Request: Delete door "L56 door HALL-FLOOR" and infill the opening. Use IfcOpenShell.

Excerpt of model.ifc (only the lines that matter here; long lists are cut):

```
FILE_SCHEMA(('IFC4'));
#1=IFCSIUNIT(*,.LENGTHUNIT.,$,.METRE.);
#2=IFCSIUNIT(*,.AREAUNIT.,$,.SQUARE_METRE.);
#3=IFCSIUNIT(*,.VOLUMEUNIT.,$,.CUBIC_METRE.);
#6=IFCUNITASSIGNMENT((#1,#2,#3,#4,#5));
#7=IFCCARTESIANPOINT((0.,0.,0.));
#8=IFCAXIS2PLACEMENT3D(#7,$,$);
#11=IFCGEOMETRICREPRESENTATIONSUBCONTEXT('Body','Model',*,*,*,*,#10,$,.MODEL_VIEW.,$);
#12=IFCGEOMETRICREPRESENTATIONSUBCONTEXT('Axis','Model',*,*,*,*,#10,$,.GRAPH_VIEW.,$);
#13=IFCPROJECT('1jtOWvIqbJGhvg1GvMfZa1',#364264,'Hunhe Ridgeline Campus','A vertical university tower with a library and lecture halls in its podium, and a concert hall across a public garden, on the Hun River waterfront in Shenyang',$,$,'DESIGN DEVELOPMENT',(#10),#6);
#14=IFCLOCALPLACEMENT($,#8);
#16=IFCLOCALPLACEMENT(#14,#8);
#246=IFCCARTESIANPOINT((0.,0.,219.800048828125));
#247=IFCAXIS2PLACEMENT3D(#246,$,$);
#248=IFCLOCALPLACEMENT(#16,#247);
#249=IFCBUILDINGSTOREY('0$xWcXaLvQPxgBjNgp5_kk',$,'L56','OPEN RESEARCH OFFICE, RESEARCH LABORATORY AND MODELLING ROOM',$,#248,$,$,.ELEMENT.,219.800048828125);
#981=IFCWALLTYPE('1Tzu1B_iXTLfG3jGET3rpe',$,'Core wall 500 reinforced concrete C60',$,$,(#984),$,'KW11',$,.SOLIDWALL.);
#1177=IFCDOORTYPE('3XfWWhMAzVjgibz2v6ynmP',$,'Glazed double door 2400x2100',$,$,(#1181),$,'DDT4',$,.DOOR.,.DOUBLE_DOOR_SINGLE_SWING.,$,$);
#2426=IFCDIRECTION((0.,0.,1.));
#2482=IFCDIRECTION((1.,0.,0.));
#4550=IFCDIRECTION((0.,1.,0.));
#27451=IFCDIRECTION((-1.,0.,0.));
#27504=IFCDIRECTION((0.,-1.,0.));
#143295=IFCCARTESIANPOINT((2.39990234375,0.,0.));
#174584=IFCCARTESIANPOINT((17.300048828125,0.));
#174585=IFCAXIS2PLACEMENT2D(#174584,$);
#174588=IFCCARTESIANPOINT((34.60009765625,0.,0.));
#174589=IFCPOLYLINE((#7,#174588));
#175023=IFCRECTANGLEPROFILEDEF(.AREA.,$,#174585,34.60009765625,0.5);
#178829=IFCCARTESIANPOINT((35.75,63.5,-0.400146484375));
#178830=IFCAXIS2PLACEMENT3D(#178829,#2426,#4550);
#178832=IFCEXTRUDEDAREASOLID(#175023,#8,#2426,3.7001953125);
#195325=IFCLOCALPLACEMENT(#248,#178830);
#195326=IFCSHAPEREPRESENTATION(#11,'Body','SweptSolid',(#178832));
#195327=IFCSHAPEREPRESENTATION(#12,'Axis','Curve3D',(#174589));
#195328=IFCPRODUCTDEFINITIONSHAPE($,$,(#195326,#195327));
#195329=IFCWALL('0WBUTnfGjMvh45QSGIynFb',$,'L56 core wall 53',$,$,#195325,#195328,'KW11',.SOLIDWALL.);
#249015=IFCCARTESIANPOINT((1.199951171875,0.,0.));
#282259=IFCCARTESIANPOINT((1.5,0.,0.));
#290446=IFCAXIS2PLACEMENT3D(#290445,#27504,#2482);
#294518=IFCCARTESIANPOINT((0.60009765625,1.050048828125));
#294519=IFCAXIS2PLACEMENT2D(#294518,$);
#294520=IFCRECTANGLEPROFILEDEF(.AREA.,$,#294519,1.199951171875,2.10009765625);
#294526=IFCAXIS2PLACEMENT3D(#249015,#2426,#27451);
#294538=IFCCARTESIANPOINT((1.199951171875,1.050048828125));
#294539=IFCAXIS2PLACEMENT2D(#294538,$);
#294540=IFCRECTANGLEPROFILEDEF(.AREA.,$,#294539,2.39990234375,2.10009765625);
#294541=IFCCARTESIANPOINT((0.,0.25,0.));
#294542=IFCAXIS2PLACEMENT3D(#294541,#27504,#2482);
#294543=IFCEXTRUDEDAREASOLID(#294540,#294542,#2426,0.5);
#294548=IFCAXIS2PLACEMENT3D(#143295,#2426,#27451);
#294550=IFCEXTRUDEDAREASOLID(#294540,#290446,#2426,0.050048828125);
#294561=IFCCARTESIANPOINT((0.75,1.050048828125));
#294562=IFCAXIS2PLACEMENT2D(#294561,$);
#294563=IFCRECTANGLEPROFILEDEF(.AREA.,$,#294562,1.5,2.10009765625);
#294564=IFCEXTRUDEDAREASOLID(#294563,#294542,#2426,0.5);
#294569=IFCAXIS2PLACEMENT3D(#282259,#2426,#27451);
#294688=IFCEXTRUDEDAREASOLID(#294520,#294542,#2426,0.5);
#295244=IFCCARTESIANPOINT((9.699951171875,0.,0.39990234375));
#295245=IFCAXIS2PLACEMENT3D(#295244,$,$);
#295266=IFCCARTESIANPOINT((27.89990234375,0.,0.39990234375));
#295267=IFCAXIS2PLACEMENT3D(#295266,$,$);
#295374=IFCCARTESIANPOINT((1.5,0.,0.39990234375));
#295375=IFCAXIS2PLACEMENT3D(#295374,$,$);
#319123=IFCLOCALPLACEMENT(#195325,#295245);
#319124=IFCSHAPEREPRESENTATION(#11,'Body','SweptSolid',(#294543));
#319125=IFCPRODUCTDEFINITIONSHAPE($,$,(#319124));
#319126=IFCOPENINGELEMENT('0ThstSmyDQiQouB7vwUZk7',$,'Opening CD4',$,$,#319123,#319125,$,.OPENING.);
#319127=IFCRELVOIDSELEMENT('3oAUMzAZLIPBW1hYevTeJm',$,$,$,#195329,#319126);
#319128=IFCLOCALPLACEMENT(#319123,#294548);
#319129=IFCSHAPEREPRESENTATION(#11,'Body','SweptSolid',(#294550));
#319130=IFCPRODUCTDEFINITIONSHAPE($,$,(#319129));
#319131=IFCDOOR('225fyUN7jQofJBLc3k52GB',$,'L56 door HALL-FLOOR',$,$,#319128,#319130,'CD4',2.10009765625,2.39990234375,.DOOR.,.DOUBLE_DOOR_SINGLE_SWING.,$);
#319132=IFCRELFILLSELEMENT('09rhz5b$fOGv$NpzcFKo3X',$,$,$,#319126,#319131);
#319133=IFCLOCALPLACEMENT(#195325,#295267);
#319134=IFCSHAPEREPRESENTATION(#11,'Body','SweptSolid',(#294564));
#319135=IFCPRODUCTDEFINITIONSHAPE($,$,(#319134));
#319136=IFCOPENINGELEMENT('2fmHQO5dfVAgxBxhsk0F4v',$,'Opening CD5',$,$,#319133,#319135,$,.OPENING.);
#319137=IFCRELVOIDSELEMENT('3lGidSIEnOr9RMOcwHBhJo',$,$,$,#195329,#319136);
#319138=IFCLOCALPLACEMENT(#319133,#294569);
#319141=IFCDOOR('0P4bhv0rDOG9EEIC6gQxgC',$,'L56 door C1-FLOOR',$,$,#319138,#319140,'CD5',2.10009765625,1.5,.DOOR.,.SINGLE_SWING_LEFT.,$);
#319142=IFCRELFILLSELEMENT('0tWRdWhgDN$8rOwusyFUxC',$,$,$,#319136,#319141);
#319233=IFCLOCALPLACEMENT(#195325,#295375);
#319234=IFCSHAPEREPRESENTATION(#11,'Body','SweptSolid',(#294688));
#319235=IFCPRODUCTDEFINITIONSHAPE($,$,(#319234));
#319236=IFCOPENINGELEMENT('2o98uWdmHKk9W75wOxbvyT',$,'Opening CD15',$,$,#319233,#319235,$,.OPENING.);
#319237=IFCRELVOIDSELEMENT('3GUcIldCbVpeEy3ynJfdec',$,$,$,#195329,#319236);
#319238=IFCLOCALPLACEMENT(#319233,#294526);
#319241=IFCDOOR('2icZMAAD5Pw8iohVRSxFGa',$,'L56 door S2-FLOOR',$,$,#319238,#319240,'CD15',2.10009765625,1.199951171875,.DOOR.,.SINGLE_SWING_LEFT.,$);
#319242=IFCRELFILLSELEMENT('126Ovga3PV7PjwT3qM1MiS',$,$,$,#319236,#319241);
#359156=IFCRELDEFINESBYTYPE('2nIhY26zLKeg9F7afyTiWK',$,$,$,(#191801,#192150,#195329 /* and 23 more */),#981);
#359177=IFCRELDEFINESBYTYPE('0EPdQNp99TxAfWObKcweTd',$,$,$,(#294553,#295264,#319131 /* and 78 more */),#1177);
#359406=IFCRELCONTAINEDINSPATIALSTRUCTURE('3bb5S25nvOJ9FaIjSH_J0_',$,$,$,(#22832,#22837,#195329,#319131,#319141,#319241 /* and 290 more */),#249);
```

```python
import ifcopenshell
import ifcopenshell.api.feature
import ifcopenshell.api.root
import ifcopenshell.geom
import ifcopenshell.util.shape

model = ifcopenshell.open("model.ifc")
settings = ifcopenshell.geom.settings()


def volume(element):
    """Net volume in cubic metres, openings subtracted."""
    shape = ifcopenshell.geom.create_shape(settings, element)
    return ifcopenshell.util.shape.get_volume(shape.geometry)


door = model.by_guid("225fyUN7jQofJBLc3k52GB")
opening = door.FillsVoids[0].RelatingOpeningElement
wall = opening.VoidsElements[0].RelatingBuildingElement
before = volume(wall)

ifcopenshell.api.root.remove_product(model, product=door)
ifcopenshell.api.feature.remove_feature(model, feature=opening)

after = volume(wall)

print(f"wall volume {before:.3f} -> {after:.3f} m3")

model.write("model_edited.ifc")
```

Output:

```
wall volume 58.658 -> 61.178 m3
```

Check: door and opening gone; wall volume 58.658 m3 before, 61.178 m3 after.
